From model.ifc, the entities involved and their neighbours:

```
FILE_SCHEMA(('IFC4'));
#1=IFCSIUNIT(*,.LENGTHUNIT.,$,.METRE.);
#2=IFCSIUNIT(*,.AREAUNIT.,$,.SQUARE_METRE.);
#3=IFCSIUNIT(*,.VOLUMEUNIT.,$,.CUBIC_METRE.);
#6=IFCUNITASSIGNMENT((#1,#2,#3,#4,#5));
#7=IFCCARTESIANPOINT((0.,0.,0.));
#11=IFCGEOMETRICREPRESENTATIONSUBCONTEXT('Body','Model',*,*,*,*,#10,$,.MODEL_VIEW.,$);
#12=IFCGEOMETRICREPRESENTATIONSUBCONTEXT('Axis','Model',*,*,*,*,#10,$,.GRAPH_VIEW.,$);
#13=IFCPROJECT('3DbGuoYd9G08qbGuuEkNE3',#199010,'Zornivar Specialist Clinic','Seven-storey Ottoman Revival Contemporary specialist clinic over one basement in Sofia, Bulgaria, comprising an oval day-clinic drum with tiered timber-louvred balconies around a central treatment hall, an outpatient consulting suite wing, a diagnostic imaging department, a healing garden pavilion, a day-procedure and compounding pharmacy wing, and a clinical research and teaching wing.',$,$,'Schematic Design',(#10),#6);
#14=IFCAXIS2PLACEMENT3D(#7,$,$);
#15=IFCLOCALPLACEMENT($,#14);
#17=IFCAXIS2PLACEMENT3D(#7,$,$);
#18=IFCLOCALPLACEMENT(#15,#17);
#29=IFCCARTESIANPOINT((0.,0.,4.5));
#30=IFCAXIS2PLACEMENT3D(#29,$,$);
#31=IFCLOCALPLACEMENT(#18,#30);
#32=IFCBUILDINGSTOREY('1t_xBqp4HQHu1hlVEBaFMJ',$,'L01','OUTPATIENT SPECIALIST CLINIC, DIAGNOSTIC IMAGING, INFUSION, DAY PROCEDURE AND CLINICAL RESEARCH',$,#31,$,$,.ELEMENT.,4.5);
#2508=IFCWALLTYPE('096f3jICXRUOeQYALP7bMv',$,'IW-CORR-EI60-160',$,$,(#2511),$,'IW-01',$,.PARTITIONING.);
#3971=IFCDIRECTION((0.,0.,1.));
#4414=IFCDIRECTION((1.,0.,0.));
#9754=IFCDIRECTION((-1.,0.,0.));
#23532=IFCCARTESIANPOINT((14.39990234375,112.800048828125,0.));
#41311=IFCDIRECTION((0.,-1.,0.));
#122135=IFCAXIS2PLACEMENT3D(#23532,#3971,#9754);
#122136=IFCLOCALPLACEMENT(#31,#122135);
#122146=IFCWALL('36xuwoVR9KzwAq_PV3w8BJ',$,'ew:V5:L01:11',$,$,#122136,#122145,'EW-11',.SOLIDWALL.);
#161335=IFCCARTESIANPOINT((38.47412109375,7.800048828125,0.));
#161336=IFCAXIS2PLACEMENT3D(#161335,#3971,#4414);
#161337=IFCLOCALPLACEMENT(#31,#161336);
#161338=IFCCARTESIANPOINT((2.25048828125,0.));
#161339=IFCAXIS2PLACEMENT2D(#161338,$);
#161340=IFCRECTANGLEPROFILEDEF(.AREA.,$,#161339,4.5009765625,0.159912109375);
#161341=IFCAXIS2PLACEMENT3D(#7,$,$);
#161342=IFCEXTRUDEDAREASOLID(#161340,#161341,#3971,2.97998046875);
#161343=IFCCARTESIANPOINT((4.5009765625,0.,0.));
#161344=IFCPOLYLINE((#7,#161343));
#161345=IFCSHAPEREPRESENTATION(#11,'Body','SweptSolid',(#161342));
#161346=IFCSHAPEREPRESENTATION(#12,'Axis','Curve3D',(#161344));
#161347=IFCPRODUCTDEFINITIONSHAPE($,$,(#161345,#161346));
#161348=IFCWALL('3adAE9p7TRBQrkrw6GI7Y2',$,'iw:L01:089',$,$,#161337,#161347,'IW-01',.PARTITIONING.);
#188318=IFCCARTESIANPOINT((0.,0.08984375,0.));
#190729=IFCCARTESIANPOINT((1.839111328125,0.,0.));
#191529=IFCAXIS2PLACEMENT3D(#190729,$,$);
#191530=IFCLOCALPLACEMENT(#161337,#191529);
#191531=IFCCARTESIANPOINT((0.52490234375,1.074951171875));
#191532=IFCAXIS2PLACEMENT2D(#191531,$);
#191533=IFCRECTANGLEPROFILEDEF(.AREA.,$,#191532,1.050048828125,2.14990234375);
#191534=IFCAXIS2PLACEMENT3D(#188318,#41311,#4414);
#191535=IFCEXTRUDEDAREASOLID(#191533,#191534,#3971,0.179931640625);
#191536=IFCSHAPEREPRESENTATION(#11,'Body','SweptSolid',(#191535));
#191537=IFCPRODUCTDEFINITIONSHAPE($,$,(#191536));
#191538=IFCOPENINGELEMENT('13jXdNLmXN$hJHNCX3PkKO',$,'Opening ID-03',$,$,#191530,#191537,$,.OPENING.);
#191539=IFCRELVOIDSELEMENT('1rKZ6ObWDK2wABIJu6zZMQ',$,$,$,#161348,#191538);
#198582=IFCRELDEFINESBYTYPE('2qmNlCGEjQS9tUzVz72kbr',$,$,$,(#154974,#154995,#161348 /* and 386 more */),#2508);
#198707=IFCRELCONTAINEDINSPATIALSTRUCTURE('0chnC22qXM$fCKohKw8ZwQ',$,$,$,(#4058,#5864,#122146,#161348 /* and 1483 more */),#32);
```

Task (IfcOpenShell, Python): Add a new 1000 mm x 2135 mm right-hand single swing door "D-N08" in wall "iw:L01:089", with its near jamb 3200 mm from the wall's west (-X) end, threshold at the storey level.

```python
import numpy as np
import ifcopenshell
import ifcopenshell.api.feature
import ifcopenshell.api.geometry
import ifcopenshell.api.root
import ifcopenshell.api.spatial
import ifcopenshell.geom
import ifcopenshell.util.element
import ifcopenshell.util.placement
import ifcopenshell.util.representation
import ifcopenshell.util.shape
import ifcopenshell.util.unit

model = ifcopenshell.open("model.ifc")
unit_scale = ifcopenshell.util.unit.calculate_unit_scale(model)
settings = ifcopenshell.geom.settings()


def volume(element):
    """Net volume in cubic metres, openings subtracted."""
    shape = ifcopenshell.geom.create_shape(settings, element)
    return ifcopenshell.util.shape.get_volume(shape.geometry)


wall = model.by_guid("3adAE9p7TRBQrkrw6GI7Y2")
storey = ifcopenshell.util.element.get_container(wall, ifc_class="IfcBuildingStorey")
context = ifcopenshell.util.representation.get_context(model, "Model", "Body", "MODEL_VIEW")
before = volume(wall)

width, height, from_end, sill = 1, 2.135, 3.2, 0.0  # metres

# The wall runs along its own X axis, and the end named is its -X end.
wall_shape = ifcopenshell.geom.create_shape(settings, wall)
x, y, z = ifcopenshell.util.shape.get_vertices(wall_shape.geometry).T
start = x.min() + from_end
face, thickness = float(y.min()), float(y.max() - y.min())
wall_matrix = ifcopenshell.util.placement.get_local_placement(wall.ObjectPlacement)
level = ifcopenshell.util.placement.get_local_placement(storey.ObjectPlacement)[2, 3]


def in_wall(x, y):
    """Placement at x, y metres in the wall's axes, at sill height."""
    matrix = wall_matrix.copy()
    matrix[:, 3] = wall_matrix @ np.array([x / unit_scale, y / unit_scale, 0.0, 1.0])
    matrix[2, 3] = level + sill / unit_scale
    return matrix


# Opening: a box that overshoots both wall faces by 50 mm.
opening = ifcopenshell.api.root.create_entity(model, ifc_class="IfcOpeningElement", predefined_type="OPENING")
box = ifcopenshell.api.geometry.add_wall_representation(
    model, context=context, length=width, height=height, thickness=thickness + 0.1
)
ifcopenshell.api.geometry.assign_representation(model, product=opening, representation=box)
ifcopenshell.api.geometry.edit_object_placement(model, product=opening, matrix=in_wall(start, face - 0.05), is_si=False)
ifcopenshell.api.feature.add_feature(model, feature=opening, element=wall)

door = ifcopenshell.api.root.create_entity(model, ifc_class="IfcDoor", name="D-N08", predefined_type="DOOR")
door.OverallWidth, door.OverallHeight = width / unit_scale, height / unit_scale
door.OperationType = "SINGLE_SWING_RIGHT"
body = ifcopenshell.api.geometry.add_door_representation(
    model,
    context=context,
    overall_width=door.OverallWidth,
    overall_height=door.OverallHeight,
    operation_type="SINGLE_SWING_RIGHT",
    lining_properties={"LiningDepth": thickness / unit_scale, "ThresholdDepth": thickness / unit_scale},
)
ifcopenshell.api.geometry.assign_representation(model, product=door, representation=body)
ifcopenshell.api.spatial.assign_container(model, products=[door], relating_structure=storey)
ifcopenshell.api.feature.add_filling(model, opening=opening, element=door)

# The lining spans the wall, so the door starts at the wall face.
ifcopenshell.api.geometry.edit_object_placement(model, product=door, matrix=in_wall(start, face), is_si=False)

after = volume(wall)

print(f"wall volume {before:.3f} -> {after:.3f} m3")

model.write("model_rev.ifc")
```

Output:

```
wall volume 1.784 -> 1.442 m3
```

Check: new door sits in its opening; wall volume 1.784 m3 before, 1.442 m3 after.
